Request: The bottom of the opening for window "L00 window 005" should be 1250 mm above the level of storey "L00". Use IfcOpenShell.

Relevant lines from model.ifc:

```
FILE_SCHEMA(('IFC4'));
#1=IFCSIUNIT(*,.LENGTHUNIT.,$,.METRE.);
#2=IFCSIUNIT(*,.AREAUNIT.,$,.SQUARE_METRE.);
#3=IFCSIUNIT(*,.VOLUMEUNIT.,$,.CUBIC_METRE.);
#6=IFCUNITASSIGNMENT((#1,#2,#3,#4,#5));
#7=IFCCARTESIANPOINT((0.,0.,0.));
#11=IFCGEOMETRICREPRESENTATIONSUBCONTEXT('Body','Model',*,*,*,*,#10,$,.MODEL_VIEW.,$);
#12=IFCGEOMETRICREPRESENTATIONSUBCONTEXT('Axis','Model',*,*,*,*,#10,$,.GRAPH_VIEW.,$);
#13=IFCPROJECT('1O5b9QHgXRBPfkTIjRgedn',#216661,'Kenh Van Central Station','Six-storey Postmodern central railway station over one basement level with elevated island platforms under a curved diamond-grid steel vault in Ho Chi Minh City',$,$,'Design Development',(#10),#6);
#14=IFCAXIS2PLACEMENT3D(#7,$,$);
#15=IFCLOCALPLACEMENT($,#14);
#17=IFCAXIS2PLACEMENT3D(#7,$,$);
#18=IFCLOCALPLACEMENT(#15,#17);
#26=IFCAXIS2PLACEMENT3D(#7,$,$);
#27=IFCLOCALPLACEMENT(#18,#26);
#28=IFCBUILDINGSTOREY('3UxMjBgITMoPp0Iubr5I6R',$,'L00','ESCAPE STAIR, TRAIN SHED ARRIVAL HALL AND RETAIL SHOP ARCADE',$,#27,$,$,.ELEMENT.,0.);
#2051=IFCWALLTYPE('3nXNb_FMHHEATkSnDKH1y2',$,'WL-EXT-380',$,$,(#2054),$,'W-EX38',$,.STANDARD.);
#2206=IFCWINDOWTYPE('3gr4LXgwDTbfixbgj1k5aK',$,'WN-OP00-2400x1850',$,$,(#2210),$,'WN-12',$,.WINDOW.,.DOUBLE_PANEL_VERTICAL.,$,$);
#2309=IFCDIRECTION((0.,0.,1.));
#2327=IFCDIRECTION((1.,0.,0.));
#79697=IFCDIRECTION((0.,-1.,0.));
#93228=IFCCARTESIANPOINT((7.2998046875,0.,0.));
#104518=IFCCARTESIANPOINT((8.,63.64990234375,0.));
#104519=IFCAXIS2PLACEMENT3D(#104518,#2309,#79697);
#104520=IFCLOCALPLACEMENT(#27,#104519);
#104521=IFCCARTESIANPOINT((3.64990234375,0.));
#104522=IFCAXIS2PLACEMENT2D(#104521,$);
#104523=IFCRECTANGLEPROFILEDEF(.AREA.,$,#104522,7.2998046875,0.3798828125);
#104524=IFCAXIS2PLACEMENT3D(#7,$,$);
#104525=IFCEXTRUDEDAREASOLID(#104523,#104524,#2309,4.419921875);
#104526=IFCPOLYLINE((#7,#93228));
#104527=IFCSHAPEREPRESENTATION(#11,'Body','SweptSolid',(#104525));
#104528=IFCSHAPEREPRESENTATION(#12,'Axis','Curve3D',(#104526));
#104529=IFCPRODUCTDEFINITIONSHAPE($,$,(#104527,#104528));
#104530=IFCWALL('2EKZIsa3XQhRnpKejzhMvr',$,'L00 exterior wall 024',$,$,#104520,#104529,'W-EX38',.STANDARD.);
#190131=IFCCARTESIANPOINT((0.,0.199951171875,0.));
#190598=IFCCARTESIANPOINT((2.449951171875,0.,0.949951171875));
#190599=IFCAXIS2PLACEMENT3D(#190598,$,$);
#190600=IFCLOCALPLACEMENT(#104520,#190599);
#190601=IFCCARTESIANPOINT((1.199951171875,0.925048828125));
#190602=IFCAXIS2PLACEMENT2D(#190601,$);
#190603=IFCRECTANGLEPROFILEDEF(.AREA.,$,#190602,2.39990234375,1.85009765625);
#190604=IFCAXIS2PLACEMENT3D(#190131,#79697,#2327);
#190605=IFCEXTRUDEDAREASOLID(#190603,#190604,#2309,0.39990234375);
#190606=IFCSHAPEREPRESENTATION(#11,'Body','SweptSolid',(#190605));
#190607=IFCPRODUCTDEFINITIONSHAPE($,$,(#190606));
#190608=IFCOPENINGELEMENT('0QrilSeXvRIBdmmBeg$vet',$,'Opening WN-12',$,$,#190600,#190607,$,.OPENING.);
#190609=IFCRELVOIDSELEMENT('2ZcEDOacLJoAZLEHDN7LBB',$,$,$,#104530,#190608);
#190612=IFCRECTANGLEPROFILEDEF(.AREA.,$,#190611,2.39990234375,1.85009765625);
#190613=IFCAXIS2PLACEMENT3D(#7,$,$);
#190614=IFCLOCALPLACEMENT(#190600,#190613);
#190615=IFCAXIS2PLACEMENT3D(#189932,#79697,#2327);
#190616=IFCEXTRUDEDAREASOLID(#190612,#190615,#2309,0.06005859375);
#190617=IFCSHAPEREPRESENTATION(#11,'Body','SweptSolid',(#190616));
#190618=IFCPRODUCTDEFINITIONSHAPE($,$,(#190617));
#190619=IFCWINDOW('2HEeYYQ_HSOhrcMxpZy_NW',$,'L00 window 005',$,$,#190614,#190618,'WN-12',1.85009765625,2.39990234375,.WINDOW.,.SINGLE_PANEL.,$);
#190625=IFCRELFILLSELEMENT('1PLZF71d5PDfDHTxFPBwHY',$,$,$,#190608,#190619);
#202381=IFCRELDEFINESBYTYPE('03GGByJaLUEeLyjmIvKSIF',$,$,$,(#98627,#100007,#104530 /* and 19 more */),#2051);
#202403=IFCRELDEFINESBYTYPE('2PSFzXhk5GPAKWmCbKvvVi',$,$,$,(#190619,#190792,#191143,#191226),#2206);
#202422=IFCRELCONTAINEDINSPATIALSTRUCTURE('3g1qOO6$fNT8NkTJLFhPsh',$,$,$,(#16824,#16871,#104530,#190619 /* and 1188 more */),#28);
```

```python
import numpy as np
import ifcopenshell
import ifcopenshell.api.geometry
import ifcopenshell.geom
import ifcopenshell.util.element
import ifcopenshell.util.placement
import ifcopenshell.util.shape
import ifcopenshell.util.unit

model = ifcopenshell.open("model.ifc")
unit_scale = ifcopenshell.util.unit.calculate_unit_scale(model)

window = model.by_guid("2HEeYYQ_HSOhrcMxpZy_NW")
opening = window.FillsVoids[0].RelatingOpeningElement
storey = ifcopenshell.util.element.get_container(window, ifc_class="IfcBuildingStorey")
level = ifcopenshell.util.placement.get_local_placement(storey.ObjectPlacement)[2, 3]

# The opening's origin need not be at the sill, so measure its lowest point.
shape = ifcopenshell.geom.create_shape(ifcopenshell.geom.settings(), opening)
bottom = ifcopenshell.util.shape.get_shape_bottom_elevation(shape, shape.geometry) / unit_scale
dz = level + 1.25 - bottom

shift = np.array([0.0, 0.0, dz])
# The window is placed relative to its opening, so it follows when the opening moves.
matrix = ifcopenshell.util.placement.get_local_placement(opening.ObjectPlacement)
matrix[:3, 3] += shift
ifcopenshell.api.geometry.edit_object_placement(
    model, product=opening, matrix=matrix, is_si=False, should_transform_children=True
)

print(f"moved by {dz * unit_scale:+.3f} m")

model.write("model_updated.ifc")
```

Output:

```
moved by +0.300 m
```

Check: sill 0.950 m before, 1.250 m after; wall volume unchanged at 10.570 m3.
